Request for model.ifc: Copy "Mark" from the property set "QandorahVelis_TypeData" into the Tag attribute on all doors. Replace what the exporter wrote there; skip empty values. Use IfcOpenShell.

First a look at what the model holds.

```python
import ifcopenshell
import ifcopenshell.util.element

model = ifcopenshell.open("model.ifc")
print(model.schema)
doors = model.by_type("IfcDoor")
print(len(doors), "doors")
for e in doors[:8]:
    source = ifcopenshell.util.element.get_pset(e, "QandorahVelis_TypeData", "Mark")
    target = e.Tag
    print(e.id(), repr(source), repr(target), sep=" | ")
```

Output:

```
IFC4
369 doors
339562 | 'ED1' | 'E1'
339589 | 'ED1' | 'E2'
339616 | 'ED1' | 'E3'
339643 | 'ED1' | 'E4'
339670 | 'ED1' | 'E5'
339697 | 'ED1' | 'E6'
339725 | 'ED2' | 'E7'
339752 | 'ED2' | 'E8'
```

```python
import ifcopenshell
import ifcopenshell.util.element

model = ifcopenshell.open("model.ifc")

count = 0
for e in model.by_type("IfcDoor"):
    value = ifcopenshell.util.element.get_pset(e, "QandorahVelis_TypeData", "Mark")
    current = e.Tag
    if not value or not value.strip() or current == value:
        continue
    e.Tag = value
    count += 1

print(count, "doors updated")

model.write("model-out.ifc")
```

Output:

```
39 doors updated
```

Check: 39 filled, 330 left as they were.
